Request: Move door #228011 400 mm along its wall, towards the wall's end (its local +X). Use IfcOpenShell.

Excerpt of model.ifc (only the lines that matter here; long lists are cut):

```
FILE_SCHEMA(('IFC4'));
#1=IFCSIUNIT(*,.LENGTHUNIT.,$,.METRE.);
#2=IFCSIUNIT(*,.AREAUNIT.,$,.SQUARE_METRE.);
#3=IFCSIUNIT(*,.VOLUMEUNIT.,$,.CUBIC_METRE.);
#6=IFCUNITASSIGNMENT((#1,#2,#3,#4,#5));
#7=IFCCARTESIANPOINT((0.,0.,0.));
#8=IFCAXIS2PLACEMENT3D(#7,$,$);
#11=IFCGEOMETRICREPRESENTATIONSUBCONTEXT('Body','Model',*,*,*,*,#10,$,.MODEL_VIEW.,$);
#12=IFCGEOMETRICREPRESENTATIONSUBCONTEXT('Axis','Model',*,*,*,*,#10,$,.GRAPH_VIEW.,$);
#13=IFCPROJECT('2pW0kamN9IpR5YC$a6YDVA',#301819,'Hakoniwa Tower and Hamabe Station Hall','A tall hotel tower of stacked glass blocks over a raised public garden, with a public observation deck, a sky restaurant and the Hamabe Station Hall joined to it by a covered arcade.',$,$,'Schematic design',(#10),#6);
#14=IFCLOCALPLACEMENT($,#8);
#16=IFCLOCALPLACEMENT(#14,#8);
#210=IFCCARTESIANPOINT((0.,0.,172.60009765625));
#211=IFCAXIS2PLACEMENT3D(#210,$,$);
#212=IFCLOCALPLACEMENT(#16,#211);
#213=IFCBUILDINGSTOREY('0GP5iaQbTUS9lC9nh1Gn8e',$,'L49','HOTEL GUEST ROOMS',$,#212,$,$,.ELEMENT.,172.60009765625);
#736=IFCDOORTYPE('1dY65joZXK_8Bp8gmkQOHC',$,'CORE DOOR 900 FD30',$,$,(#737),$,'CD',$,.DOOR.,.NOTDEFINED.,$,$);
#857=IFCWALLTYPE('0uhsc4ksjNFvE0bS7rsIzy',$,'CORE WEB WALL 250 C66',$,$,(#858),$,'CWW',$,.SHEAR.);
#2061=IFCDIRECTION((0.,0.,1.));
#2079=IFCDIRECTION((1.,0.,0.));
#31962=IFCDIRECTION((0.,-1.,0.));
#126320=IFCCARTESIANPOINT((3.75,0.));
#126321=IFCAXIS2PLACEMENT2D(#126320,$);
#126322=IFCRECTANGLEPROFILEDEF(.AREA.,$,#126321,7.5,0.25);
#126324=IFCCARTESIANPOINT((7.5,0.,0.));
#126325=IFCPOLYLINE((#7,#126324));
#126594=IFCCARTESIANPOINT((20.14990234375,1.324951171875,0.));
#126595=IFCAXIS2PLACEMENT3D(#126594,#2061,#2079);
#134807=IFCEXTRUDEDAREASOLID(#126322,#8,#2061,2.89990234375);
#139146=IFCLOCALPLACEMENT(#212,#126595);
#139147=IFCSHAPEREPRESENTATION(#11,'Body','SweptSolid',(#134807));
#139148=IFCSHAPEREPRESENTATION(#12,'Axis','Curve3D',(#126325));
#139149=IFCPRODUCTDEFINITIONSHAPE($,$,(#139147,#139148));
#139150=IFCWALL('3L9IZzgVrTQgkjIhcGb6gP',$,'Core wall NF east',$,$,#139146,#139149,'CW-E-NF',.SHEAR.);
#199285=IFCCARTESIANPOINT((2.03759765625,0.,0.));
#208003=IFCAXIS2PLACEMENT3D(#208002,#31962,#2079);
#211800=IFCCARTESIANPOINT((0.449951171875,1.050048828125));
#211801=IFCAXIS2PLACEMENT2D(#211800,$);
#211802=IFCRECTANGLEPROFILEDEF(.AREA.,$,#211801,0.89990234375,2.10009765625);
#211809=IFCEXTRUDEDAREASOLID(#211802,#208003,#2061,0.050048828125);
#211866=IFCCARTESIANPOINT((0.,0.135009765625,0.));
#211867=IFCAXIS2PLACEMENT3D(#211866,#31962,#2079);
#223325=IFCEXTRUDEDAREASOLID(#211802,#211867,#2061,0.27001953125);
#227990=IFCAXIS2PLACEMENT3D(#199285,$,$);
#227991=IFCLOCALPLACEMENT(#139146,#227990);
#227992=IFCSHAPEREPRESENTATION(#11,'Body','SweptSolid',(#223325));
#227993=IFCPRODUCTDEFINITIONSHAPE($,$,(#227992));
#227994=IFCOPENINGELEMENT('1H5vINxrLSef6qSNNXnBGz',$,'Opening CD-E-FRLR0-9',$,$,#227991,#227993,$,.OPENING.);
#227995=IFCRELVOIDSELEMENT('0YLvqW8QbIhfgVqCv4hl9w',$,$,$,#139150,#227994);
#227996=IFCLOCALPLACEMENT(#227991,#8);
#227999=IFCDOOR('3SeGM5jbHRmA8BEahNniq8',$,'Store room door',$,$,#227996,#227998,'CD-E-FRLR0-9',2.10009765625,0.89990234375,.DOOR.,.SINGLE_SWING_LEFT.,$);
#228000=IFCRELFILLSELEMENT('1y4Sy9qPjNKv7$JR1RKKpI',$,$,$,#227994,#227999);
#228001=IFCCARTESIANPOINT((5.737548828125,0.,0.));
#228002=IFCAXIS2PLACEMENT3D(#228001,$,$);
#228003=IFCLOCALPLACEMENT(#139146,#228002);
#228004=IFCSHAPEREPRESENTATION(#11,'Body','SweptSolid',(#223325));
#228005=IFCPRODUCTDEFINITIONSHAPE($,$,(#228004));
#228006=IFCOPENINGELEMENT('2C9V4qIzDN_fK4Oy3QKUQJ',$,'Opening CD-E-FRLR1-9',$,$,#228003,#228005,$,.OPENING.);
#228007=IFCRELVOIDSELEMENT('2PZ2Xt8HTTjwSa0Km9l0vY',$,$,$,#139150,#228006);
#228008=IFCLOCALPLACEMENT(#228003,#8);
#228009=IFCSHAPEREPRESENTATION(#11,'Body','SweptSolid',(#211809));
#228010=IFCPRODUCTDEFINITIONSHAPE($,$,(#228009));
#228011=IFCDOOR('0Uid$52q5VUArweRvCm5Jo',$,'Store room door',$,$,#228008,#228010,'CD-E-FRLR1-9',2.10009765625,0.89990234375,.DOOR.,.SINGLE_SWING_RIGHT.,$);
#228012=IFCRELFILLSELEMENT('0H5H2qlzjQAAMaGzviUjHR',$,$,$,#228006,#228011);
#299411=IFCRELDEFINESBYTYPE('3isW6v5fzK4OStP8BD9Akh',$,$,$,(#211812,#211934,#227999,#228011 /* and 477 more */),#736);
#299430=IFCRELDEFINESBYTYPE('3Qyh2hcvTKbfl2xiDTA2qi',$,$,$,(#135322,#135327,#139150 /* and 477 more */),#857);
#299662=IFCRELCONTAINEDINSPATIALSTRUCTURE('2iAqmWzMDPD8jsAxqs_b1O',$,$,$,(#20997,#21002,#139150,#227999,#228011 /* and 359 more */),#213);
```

```python
import ifcopenshell
import ifcopenshell.api.geometry
import ifcopenshell.util.placement

model = ifcopenshell.open("model.ifc")

door = model.by_id(228011)
opening = door.FillsVoids[0].RelatingOpeningElement
wall = opening.VoidsElements[0].RelatingBuildingElement

wall_matrix = ifcopenshell.util.placement.get_local_placement(wall.ObjectPlacement)
shift = wall_matrix[:3, 0] * 0.4
before = ifcopenshell.util.placement.get_local_placement(door.ObjectPlacement)[:3, 3].copy()

# The door is placed relative to its opening, so it follows when the opening moves.
matrix = ifcopenshell.util.placement.get_local_placement(opening.ObjectPlacement)
matrix[:3, 3] += shift
ifcopenshell.api.geometry.edit_object_placement(
    model, product=opening, matrix=matrix, is_si=False, should_transform_children=True
)

after = ifcopenshell.util.placement.get_local_placement(door.ObjectPlacement)[:3, 3]
print("door moved by", (after - before).round(3) + 0.0)

model.write("model_v2.ifc")
```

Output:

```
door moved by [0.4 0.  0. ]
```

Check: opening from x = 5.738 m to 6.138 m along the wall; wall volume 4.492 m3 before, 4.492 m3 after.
